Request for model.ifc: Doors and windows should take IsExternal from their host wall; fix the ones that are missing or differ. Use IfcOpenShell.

First a look at what the model holds.

```python
import ifcopenshell
import ifcopenshell.util.element

model = ifcopenshell.open("model.ifc")
print(model.schema)
seen = {}
for e in model.by_type("IfcDoor") + model.by_type("IfcWindow"):
    if not e.FillsVoids:
        continue
    host = e.FillsVoids[0].RelatingOpeningElement.VoidsElements[0].RelatingBuildingElement
    own = ifcopenshell.util.element.get_pset(e, f"Pset_{e.is_a()[3:].removesuffix('StandardCase')}Common", "IsExternal")
    wall = ifcopenshell.util.element.get_pset(host, "Pset_WallCommon", "IsExternal")
    seen[e.is_a(), own, wall] = seen.get((e.is_a(), own, wall), 0) + 1
for (cls, own, wall), count in sorted(seen.items(), key=str):
    print(count, cls, "IsExternal:", own, "| host wall:", wall)
```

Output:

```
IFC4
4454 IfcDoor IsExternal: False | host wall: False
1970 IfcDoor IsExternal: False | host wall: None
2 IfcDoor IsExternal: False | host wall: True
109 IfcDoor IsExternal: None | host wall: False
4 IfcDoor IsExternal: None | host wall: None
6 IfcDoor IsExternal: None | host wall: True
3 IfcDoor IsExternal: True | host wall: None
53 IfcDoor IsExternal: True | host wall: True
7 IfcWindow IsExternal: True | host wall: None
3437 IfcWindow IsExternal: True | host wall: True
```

```python
import ifcopenshell
import ifcopenshell.api.pset
import ifcopenshell.util.element

model = ifcopenshell.open("model.ifc")

count = 0
for ifc_class, pset_name in (("IfcDoor", "Pset_DoorCommon"), ("IfcWindow", "Pset_WindowCommon")):
    for e in model.by_type(ifc_class):
        if not e.FillsVoids:
            continue
        host = e.FillsVoids[0].RelatingOpeningElement.VoidsElements[0].RelatingBuildingElement
        external = ifcopenshell.util.element.get_pset(host, "Pset_WallCommon", "IsExternal")
        if external is None or ifcopenshell.util.element.get_pset(e, pset_name, "IsExternal") == external:
            continue
        found = ifcopenshell.util.element.get_pset(e, pset_name, should_inherit=False)
        if found:
            pset = model.by_id(found["id"])
            if len(ifcopenshell.util.element.get_elements_by_pset(pset)) > 1:
                pset = ifcopenshell.api.pset.unshare_pset(model, products=[e], pset=pset)[0]
        else:
            pset = ifcopenshell.api.pset.add_pset(model, product=e, name=pset_name)
        ifcopenshell.api.pset.edit_pset(model, pset=pset, properties={"IsExternal": external})
        count += 1

print(count, "updated")

model.write("model_updated.ifc")
```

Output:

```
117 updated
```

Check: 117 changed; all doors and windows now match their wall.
